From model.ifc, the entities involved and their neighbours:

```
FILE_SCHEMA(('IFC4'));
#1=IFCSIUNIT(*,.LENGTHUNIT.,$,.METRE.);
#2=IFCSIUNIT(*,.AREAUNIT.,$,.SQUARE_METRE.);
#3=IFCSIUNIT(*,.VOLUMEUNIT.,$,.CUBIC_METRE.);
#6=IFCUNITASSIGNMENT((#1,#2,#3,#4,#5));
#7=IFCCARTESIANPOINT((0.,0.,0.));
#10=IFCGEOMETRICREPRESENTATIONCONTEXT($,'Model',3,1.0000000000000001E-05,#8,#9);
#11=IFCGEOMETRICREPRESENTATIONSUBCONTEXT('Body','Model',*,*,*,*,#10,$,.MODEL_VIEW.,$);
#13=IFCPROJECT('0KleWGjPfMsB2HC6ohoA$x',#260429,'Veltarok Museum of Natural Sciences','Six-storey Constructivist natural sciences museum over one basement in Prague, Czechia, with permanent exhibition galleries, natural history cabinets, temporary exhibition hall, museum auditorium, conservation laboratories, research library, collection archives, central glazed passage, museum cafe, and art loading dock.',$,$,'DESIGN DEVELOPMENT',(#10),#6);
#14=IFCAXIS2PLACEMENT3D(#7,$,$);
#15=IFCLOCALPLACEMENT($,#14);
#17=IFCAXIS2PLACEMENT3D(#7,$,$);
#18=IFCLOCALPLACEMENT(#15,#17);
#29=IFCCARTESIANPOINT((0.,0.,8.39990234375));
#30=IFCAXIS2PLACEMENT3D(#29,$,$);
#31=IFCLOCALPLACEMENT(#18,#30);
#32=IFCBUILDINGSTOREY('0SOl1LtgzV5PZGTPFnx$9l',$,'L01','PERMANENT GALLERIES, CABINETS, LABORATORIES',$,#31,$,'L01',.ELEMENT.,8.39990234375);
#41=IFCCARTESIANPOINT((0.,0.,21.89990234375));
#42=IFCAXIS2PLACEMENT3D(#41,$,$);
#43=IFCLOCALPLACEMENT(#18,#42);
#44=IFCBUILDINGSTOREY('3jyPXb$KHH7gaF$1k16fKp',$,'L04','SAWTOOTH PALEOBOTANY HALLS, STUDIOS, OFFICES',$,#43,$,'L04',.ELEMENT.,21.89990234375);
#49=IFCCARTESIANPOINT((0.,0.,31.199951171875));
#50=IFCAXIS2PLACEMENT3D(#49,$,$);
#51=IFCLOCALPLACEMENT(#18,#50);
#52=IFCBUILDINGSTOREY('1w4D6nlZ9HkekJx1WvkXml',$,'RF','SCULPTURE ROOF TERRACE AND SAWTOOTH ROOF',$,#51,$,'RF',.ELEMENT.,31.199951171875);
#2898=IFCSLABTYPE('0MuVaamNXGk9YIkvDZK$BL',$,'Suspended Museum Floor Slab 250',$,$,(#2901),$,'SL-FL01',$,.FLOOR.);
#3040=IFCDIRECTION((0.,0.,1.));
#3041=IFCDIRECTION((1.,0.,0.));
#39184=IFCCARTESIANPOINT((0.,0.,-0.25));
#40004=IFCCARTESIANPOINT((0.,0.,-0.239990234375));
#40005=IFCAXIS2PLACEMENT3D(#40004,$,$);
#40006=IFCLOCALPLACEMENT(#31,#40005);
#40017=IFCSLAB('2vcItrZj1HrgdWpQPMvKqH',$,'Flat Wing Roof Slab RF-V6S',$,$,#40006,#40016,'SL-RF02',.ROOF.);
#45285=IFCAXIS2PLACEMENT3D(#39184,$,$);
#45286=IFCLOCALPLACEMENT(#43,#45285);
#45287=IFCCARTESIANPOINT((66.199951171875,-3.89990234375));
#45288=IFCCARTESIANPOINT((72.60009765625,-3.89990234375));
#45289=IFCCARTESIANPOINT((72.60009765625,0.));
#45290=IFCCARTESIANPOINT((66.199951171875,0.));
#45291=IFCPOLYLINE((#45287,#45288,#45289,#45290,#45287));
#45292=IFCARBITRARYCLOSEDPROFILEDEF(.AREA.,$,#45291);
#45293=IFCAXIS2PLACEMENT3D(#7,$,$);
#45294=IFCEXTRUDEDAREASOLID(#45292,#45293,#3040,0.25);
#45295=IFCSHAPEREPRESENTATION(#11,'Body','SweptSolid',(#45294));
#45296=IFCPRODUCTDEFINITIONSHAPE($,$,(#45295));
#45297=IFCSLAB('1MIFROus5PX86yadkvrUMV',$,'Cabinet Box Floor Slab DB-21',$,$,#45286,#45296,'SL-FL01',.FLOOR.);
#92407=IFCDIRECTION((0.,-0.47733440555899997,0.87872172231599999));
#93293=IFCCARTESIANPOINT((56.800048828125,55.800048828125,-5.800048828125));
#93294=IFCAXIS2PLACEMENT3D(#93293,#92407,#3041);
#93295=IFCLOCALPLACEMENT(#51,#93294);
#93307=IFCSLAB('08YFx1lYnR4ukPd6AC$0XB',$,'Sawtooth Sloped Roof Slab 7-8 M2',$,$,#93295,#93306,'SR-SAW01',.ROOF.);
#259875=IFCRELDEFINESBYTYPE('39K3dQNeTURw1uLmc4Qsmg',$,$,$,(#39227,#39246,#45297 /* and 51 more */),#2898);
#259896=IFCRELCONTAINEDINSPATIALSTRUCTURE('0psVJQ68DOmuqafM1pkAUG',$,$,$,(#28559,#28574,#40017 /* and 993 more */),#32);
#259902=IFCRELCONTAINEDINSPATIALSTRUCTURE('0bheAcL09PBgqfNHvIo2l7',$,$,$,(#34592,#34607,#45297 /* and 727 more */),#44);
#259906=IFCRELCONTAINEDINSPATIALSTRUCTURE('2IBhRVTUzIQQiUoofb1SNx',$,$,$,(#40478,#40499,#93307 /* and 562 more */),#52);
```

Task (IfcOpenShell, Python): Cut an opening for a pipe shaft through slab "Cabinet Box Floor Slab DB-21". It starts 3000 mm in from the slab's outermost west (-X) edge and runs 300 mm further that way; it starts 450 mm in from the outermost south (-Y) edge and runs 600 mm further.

```python
import numpy as np
import ifcopenshell
import ifcopenshell.api.feature
import ifcopenshell.api.geometry
import ifcopenshell.api.root
import ifcopenshell.geom
import ifcopenshell.util.placement
import ifcopenshell.util.representation
import ifcopenshell.util.shape
import ifcopenshell.util.unit

model = ifcopenshell.open("model.ifc")
unit_scale = ifcopenshell.util.unit.calculate_unit_scale(model)
settings = ifcopenshell.geom.settings()


def volume(element):
    """Net volume in cubic metres, openings subtracted."""
    shape = ifcopenshell.geom.create_shape(settings, element)
    return ifcopenshell.util.shape.get_volume(shape.geometry)


slab = model.by_id(45297)
before = volume(slab)

# Extent in the slab's own axes, in metres. The edges named are its -X and -Y sides.
slab_shape = ifcopenshell.geom.create_shape(settings, slab)
vertices = ifcopenshell.util.shape.get_vertices(slab_shape.geometry)
x_min, y_min, bottom = vertices.min(axis=0)
top = vertices[:, 2].max()

opening = ifcopenshell.api.root.create_entity(model, ifc_class="IfcOpeningElement", name="Pipe shaft opening", predefined_type="OPENING")
context = ifcopenshell.util.representation.get_context(model, "Model", "Body", "MODEL_VIEW")
width, depth = 0.3, 0.6
outline = [(0.0, 0.0), (width, 0.0), (width, depth), (0.0, depth), (0.0, 0.0)]
# Overshoot both faces by 50 mm so the cut is clean.
shape = ifcopenshell.api.geometry.add_slab_representation(
    model, context=context, depth=top - bottom + 0.1, polyline=outline
)
ifcopenshell.api.geometry.assign_representation(model, product=opening, representation=shape)

matrix = ifcopenshell.util.placement.get_local_placement(slab.ObjectPlacement)
matrix[:, 3] = matrix @ np.append(np.array([x_min + 3, y_min + 0.45, bottom - 0.05]) / unit_scale, 1.0)
ifcopenshell.api.geometry.edit_object_placement(model, product=opening, matrix=matrix, is_si=False)
ifcopenshell.api.feature.add_feature(model, feature=opening, element=slab)

after = volume(slab)

print(f"slab volume {before:.3f} -> {after:.3f} m3")

model.write("model-out.ifc")
```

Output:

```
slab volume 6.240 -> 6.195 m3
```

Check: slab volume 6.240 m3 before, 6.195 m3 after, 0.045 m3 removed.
